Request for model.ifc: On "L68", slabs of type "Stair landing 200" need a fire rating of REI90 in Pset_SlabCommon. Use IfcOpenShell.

First a look at what the model holds.

```python
import ifcopenshell
import ifcopenshell.util.element

model = ifcopenshell.open("model.ifc")
print(model.schema)
storey = next(s for s in model.by_type("IfcBuildingStorey") if s.Name == "L68")
slabs = [e for e in ifcopenshell.util.element.get_decomposition(storey) if e.is_a("IfcSlab")]
seen = {}
for e in slabs:
    element_type = ifcopenshell.util.element.get_type(e)
    key = (element_type.Name if element_type != e and element_type else None, ifcopenshell.util.element.get_pset(e, "Pset_SlabCommon", "FireRating"))
    seen[key] = seen.get(key, 0) + 1
for (name, value), count in sorted(seen.items(), key=str):
    print(count, "x", name, "|", value)
```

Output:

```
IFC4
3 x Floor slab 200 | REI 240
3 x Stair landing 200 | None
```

```python
import ifcopenshell
import ifcopenshell.api.pset
import ifcopenshell.util.element

model = ifcopenshell.open("model.ifc")

storey = next(s for s in model.by_type("IfcBuildingStorey") if s.Name == "L68")
slabs = [e for e in ifcopenshell.util.element.get_decomposition(storey) if e.is_a("IfcSlab")]

count = 0
for e in slabs:
    element_type = ifcopenshell.util.element.get_type(e)
    if element_type in (None, e) or element_type.Name != "Stair landing 200":
        continue
    found = ifcopenshell.util.element.get_pset(e, "Pset_SlabCommon", should_inherit=False)
    if found:
        pset = model.by_id(found["id"])
        if len(ifcopenshell.util.element.get_elements_by_pset(pset)) > 1:
            pset = ifcopenshell.api.pset.unshare_pset(model, products=[e], pset=pset)[0]
    else:
        pset = ifcopenshell.api.pset.add_pset(model, product=e, name="Pset_SlabCommon")
    ifcopenshell.api.pset.edit_pset(model, pset=pset, properties={"FireRating": "REI90"})
    count += 1

print(count, "slabs updated")

model.write("model_v2.ifc")
```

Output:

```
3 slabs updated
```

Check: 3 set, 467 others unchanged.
